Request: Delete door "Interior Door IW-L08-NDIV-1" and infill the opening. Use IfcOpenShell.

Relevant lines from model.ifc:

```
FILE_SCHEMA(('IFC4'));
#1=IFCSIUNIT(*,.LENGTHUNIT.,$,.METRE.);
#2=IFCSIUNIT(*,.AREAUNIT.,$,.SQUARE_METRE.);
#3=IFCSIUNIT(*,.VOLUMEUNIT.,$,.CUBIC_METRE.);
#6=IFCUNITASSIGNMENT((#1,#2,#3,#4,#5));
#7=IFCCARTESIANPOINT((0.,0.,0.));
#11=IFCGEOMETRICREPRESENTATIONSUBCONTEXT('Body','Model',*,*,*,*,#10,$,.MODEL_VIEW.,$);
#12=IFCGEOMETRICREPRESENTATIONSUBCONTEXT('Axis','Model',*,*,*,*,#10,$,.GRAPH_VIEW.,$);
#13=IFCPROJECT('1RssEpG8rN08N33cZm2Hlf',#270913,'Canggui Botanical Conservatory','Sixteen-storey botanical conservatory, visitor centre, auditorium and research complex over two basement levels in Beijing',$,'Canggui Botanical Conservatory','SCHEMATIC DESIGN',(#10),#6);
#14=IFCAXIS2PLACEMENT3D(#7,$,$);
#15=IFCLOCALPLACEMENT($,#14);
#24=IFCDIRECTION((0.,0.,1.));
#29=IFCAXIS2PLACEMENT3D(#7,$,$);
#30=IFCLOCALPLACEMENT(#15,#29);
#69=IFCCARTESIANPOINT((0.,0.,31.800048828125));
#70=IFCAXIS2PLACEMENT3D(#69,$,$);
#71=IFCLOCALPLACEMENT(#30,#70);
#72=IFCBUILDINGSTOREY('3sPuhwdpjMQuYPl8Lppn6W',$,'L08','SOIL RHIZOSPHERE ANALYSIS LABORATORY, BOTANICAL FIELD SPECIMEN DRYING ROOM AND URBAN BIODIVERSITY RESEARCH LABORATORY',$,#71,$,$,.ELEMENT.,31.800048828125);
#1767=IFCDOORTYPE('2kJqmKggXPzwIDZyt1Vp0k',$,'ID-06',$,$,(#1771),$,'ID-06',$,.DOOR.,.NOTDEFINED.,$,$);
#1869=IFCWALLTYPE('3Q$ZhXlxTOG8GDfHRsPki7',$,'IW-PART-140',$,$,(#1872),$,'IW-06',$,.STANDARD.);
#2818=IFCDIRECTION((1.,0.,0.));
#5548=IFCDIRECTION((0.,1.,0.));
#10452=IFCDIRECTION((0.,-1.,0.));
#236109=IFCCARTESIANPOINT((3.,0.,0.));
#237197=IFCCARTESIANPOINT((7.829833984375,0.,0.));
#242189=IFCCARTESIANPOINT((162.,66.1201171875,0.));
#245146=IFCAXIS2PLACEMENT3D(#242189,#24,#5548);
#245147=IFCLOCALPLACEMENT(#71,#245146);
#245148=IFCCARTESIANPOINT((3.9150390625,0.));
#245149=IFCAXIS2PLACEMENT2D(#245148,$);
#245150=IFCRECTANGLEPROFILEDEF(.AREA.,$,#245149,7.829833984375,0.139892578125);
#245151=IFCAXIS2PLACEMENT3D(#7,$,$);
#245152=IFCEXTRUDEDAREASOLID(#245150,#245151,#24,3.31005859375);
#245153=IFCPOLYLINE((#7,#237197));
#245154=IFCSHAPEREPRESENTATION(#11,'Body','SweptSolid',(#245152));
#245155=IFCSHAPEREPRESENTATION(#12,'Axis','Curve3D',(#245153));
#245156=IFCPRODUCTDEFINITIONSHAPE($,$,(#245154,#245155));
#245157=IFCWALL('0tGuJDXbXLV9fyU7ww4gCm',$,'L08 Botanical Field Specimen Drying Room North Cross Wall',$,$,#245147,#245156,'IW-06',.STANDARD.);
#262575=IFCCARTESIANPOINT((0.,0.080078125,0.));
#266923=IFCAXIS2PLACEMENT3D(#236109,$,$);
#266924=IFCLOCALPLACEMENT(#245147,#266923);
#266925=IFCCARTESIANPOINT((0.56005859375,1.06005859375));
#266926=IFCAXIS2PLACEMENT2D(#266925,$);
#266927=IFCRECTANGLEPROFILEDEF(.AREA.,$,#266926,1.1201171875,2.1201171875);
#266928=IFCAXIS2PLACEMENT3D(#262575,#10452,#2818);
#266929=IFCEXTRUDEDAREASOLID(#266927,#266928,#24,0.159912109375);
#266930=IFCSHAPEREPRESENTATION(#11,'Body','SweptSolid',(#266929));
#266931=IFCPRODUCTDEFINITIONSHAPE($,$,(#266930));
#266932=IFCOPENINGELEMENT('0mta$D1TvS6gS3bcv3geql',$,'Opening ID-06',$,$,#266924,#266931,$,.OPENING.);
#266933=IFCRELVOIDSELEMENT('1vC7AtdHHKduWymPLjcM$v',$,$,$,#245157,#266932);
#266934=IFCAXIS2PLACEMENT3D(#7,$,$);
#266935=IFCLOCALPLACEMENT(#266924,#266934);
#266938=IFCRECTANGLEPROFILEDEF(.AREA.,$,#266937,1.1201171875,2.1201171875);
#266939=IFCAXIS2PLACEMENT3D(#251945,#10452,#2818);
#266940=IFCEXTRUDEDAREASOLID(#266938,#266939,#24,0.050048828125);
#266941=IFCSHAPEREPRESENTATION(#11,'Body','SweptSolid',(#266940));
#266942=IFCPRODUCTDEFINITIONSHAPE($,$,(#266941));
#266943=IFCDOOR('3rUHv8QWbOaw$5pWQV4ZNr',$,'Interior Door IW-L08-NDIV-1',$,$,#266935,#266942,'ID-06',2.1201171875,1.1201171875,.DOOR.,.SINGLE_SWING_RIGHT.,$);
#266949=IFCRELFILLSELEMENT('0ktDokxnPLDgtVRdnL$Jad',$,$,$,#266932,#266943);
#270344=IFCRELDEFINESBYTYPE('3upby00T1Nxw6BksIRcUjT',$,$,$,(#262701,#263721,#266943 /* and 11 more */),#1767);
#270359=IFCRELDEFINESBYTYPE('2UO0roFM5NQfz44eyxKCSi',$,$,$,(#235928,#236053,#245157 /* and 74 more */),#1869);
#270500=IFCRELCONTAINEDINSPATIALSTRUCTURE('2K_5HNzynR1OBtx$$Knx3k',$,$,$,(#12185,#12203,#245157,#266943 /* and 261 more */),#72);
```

```python
import ifcopenshell
import ifcopenshell.api.feature
import ifcopenshell.api.root
import ifcopenshell.geom
import ifcopenshell.util.shape

model = ifcopenshell.open("model.ifc")
settings = ifcopenshell.geom.settings()


def volume(element):
    """Net volume in cubic metres, openings subtracted."""
    shape = ifcopenshell.geom.create_shape(settings, element)
    return ifcopenshell.util.shape.get_volume(shape.geometry)


door = model.by_guid("3rUHv8QWbOaw$5pWQV4ZNr")
opening = door.FillsVoids[0].RelatingOpeningElement
wall = opening.VoidsElements[0].RelatingBuildingElement
before = volume(wall)

ifcopenshell.api.root.remove_product(model, product=door)
ifcopenshell.api.feature.remove_feature(model, feature=opening)

after = volume(wall)

print(f"wall volume {before:.3f} -> {after:.3f} m3")

model.write("model_edited.ifc")
```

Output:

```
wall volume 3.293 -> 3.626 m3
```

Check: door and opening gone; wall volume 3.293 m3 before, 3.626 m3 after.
